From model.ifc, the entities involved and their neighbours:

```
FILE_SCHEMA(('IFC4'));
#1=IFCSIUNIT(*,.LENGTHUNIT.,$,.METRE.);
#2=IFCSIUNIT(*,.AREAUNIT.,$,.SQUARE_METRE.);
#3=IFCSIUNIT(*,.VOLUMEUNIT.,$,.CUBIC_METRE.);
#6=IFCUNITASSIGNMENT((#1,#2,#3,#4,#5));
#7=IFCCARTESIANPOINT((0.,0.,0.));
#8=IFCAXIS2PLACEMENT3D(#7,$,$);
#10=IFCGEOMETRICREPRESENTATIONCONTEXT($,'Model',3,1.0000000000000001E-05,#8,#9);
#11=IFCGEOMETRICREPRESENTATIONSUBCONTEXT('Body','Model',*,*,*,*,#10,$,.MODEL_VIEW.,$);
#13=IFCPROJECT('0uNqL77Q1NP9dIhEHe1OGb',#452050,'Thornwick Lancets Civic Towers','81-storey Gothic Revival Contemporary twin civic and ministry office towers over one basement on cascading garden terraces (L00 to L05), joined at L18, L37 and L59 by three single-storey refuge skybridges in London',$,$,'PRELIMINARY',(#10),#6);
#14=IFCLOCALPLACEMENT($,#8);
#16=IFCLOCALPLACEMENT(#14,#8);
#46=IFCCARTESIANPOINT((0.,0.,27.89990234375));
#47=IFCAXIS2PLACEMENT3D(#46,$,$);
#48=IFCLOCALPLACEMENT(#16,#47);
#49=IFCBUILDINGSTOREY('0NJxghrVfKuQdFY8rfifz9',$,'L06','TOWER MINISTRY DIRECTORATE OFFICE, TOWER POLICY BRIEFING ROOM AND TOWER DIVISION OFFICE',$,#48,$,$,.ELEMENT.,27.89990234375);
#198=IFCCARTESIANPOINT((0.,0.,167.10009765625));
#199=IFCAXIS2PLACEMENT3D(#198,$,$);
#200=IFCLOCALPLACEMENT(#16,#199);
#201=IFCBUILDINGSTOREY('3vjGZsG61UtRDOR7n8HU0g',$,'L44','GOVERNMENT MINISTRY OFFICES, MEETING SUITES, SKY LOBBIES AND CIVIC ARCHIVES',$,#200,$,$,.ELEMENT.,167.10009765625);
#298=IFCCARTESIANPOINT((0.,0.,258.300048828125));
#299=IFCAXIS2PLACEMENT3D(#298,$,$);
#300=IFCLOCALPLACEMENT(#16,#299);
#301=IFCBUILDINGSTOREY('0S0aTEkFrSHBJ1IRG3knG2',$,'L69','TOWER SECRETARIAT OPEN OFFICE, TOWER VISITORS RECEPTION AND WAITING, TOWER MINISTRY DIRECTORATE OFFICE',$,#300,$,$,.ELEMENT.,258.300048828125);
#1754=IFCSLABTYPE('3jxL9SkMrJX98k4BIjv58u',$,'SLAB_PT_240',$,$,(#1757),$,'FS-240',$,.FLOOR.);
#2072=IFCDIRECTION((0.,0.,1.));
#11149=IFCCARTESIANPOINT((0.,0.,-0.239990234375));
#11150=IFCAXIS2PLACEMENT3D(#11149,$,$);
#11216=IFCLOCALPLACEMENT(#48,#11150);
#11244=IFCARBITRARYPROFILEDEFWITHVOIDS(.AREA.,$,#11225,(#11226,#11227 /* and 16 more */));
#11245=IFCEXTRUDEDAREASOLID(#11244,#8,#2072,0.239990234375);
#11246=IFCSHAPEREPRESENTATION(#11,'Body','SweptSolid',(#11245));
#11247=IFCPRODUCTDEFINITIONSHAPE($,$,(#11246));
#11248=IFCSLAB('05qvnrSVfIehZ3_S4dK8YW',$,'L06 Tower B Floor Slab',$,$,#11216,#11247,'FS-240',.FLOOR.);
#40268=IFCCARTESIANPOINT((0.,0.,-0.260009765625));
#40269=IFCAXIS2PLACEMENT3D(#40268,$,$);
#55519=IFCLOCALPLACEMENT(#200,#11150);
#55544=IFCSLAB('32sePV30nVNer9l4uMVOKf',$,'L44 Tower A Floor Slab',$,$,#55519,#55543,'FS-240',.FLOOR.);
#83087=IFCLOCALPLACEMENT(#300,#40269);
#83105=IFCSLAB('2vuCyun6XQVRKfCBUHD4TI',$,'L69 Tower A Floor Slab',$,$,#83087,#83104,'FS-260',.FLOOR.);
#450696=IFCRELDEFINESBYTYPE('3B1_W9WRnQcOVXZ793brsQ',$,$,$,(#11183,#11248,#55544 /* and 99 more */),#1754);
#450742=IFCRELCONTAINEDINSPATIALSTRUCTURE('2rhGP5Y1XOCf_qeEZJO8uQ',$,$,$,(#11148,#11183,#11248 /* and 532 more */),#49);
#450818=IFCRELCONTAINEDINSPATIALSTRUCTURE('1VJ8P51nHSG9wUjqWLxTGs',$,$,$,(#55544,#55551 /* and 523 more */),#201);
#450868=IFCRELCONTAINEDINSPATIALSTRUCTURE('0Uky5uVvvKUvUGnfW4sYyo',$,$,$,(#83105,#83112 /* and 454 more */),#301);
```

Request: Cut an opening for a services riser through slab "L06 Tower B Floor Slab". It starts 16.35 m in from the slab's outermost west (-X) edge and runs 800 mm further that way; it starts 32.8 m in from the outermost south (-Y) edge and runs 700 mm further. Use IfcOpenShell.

```python
import numpy as np
import ifcopenshell
import ifcopenshell.api.feature
import ifcopenshell.api.geometry
import ifcopenshell.api.root
import ifcopenshell.geom
import ifcopenshell.util.placement
import ifcopenshell.util.representation
import ifcopenshell.util.shape
import ifcopenshell.util.unit

model = ifcopenshell.open("model.ifc")
unit_scale = ifcopenshell.util.unit.calculate_unit_scale(model)
settings = ifcopenshell.geom.settings()


def volume(element):
    """Net volume in cubic metres, openings subtracted."""
    shape = ifcopenshell.geom.create_shape(settings, element)
    return ifcopenshell.util.shape.get_volume(shape.geometry)


slab = model.by_guid("05qvnrSVfIehZ3_S4dK8YW")
before = volume(slab)

# Extent in the slab's own axes, in metres. The edges named are its -X and -Y sides.
slab_shape = ifcopenshell.geom.create_shape(settings, slab)
vertices = ifcopenshell.util.shape.get_vertices(slab_shape.geometry)
x_min, y_min, bottom = vertices.min(axis=0)
top = vertices[:, 2].max()

opening = ifcopenshell.api.root.create_entity(model, ifc_class="IfcOpeningElement", name="Services riser opening", predefined_type="OPENING")
context = ifcopenshell.util.representation.get_context(model, "Model", "Body", "MODEL_VIEW")
width, depth = 0.8, 0.7
outline = [(0.0, 0.0), (width, 0.0), (width, depth), (0.0, depth), (0.0, 0.0)]
# Overshoot both faces by 50 mm so the cut is clean.
shape = ifcopenshell.api.geometry.add_slab_representation(
    model, context=context, depth=top - bottom + 0.1, polyline=outline
)
ifcopenshell.api.geometry.assign_representation(model, product=opening, representation=shape)

matrix = ifcopenshell.util.placement.get_local_placement(slab.ObjectPlacement)
matrix[:, 3] = matrix @ np.append(np.array([x_min + 16.35, y_min + 32.8, bottom - 0.05]) / unit_scale, 1.0)
ifcopenshell.api.geometry.edit_object_placement(model, product=opening, matrix=matrix, is_si=False)
ifcopenshell.api.feature.add_feature(model, feature=opening, element=slab)

after = volume(slab)

print(f"slab volume {before:.3f} -> {after:.3f} m3")

model.write("model_updated.ifc")
```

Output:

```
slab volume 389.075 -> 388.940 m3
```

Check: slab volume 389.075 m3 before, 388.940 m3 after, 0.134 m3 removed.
